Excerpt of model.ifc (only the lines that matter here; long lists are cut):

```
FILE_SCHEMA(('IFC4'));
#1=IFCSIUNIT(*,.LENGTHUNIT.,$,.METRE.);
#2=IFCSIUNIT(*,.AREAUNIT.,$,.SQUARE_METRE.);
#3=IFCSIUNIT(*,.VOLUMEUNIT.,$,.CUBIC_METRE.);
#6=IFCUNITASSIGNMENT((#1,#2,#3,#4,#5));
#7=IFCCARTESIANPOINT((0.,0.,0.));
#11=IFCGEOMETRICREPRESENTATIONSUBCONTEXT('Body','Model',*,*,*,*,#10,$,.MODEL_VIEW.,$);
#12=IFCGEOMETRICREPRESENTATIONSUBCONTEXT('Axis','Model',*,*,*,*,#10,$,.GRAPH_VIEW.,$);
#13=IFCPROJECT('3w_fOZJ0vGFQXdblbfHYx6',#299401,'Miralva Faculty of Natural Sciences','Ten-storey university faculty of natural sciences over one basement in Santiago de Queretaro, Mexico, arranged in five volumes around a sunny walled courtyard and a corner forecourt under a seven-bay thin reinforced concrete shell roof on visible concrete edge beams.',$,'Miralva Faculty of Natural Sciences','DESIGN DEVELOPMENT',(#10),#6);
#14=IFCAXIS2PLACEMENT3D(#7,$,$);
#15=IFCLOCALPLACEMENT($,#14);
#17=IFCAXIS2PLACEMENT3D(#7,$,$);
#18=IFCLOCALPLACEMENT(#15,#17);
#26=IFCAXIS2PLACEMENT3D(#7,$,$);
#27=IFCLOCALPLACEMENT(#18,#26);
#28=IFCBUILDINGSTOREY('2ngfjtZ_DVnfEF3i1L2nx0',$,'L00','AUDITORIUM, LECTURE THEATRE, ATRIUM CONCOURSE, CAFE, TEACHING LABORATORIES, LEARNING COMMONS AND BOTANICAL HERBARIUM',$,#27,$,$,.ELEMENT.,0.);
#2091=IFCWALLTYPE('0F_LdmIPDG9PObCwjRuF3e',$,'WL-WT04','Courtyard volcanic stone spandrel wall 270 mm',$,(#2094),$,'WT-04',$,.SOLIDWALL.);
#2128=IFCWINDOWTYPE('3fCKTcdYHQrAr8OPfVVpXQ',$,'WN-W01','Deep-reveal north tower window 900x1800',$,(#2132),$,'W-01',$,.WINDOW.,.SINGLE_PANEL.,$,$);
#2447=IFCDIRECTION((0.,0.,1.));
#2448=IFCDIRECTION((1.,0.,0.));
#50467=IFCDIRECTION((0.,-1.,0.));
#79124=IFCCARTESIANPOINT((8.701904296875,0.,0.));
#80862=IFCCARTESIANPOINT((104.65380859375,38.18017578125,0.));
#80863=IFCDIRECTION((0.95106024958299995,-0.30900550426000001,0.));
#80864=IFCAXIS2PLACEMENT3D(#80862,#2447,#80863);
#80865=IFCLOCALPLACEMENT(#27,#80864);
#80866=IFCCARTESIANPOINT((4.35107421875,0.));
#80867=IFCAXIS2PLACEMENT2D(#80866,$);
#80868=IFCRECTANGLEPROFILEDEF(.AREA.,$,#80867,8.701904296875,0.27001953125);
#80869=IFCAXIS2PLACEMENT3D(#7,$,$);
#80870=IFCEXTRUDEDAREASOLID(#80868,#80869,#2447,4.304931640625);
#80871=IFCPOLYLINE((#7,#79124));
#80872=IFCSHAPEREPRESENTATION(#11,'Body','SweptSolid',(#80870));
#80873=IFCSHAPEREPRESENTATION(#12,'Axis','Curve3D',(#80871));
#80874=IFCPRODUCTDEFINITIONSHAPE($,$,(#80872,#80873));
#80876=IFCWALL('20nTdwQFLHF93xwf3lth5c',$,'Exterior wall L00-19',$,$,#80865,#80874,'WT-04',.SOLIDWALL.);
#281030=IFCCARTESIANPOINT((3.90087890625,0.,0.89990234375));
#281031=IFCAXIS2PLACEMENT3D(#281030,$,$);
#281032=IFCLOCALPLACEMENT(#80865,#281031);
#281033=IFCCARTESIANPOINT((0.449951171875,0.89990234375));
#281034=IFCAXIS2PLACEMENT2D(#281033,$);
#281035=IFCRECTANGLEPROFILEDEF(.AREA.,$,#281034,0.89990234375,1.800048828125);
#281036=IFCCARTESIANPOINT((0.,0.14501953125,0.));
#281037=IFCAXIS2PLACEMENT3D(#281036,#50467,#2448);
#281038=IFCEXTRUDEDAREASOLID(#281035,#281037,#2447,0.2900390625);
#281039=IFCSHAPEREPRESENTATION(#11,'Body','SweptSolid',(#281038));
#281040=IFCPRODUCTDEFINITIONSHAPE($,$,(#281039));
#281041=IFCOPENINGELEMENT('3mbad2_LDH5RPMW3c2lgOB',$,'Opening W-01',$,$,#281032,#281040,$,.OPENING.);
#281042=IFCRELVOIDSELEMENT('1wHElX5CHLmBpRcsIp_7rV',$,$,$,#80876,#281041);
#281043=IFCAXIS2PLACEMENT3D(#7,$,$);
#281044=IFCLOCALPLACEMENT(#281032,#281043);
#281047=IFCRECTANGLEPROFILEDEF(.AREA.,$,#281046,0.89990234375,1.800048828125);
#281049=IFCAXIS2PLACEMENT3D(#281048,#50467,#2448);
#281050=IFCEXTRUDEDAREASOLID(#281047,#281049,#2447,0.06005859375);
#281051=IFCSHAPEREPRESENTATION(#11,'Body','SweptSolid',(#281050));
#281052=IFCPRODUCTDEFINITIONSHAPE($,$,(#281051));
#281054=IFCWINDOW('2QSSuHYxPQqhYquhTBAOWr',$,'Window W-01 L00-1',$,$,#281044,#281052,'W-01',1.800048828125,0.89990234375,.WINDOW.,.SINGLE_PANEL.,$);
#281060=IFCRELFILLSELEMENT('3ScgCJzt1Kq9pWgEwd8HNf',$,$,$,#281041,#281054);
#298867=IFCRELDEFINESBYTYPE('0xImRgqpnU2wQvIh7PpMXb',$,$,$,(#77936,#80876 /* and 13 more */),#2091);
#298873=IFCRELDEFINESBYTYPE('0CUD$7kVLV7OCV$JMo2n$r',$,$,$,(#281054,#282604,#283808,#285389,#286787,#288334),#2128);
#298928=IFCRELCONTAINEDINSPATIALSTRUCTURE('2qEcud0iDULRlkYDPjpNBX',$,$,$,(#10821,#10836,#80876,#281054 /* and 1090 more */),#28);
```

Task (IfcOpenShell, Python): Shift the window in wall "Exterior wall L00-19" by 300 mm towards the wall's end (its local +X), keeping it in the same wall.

```python
import ifcopenshell
import ifcopenshell.api.geometry
import ifcopenshell.util.placement
import ifcopenshell.util.unit

model = ifcopenshell.open("model.ifc")
unit_scale = ifcopenshell.util.unit.calculate_unit_scale(model)

window = model.by_guid("2QSSuHYxPQqhYquhTBAOWr")
opening = window.FillsVoids[0].RelatingOpeningElement
wall = opening.VoidsElements[0].RelatingBuildingElement

wall_matrix = ifcopenshell.util.placement.get_local_placement(wall.ObjectPlacement)
shift = wall_matrix[:3, 0] * 0.3 / unit_scale
before = ifcopenshell.util.placement.get_local_placement(window.ObjectPlacement)[:3, 3].copy()

# The window is placed relative to its opening, so it follows when the opening moves.
matrix = ifcopenshell.util.placement.get_local_placement(opening.ObjectPlacement)
matrix[:3, 3] += shift
ifcopenshell.api.geometry.edit_object_placement(
    model, product=opening, matrix=matrix, is_si=False, should_transform_children=True
)

after = ifcopenshell.util.placement.get_local_placement(window.ObjectPlacement)[:3, 3]
print("window moved by", (after - before).round(3) + 0.0)

model.write("model_edited.ifc")
```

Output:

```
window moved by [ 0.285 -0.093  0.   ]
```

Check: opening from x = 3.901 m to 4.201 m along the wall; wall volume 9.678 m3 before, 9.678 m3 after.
